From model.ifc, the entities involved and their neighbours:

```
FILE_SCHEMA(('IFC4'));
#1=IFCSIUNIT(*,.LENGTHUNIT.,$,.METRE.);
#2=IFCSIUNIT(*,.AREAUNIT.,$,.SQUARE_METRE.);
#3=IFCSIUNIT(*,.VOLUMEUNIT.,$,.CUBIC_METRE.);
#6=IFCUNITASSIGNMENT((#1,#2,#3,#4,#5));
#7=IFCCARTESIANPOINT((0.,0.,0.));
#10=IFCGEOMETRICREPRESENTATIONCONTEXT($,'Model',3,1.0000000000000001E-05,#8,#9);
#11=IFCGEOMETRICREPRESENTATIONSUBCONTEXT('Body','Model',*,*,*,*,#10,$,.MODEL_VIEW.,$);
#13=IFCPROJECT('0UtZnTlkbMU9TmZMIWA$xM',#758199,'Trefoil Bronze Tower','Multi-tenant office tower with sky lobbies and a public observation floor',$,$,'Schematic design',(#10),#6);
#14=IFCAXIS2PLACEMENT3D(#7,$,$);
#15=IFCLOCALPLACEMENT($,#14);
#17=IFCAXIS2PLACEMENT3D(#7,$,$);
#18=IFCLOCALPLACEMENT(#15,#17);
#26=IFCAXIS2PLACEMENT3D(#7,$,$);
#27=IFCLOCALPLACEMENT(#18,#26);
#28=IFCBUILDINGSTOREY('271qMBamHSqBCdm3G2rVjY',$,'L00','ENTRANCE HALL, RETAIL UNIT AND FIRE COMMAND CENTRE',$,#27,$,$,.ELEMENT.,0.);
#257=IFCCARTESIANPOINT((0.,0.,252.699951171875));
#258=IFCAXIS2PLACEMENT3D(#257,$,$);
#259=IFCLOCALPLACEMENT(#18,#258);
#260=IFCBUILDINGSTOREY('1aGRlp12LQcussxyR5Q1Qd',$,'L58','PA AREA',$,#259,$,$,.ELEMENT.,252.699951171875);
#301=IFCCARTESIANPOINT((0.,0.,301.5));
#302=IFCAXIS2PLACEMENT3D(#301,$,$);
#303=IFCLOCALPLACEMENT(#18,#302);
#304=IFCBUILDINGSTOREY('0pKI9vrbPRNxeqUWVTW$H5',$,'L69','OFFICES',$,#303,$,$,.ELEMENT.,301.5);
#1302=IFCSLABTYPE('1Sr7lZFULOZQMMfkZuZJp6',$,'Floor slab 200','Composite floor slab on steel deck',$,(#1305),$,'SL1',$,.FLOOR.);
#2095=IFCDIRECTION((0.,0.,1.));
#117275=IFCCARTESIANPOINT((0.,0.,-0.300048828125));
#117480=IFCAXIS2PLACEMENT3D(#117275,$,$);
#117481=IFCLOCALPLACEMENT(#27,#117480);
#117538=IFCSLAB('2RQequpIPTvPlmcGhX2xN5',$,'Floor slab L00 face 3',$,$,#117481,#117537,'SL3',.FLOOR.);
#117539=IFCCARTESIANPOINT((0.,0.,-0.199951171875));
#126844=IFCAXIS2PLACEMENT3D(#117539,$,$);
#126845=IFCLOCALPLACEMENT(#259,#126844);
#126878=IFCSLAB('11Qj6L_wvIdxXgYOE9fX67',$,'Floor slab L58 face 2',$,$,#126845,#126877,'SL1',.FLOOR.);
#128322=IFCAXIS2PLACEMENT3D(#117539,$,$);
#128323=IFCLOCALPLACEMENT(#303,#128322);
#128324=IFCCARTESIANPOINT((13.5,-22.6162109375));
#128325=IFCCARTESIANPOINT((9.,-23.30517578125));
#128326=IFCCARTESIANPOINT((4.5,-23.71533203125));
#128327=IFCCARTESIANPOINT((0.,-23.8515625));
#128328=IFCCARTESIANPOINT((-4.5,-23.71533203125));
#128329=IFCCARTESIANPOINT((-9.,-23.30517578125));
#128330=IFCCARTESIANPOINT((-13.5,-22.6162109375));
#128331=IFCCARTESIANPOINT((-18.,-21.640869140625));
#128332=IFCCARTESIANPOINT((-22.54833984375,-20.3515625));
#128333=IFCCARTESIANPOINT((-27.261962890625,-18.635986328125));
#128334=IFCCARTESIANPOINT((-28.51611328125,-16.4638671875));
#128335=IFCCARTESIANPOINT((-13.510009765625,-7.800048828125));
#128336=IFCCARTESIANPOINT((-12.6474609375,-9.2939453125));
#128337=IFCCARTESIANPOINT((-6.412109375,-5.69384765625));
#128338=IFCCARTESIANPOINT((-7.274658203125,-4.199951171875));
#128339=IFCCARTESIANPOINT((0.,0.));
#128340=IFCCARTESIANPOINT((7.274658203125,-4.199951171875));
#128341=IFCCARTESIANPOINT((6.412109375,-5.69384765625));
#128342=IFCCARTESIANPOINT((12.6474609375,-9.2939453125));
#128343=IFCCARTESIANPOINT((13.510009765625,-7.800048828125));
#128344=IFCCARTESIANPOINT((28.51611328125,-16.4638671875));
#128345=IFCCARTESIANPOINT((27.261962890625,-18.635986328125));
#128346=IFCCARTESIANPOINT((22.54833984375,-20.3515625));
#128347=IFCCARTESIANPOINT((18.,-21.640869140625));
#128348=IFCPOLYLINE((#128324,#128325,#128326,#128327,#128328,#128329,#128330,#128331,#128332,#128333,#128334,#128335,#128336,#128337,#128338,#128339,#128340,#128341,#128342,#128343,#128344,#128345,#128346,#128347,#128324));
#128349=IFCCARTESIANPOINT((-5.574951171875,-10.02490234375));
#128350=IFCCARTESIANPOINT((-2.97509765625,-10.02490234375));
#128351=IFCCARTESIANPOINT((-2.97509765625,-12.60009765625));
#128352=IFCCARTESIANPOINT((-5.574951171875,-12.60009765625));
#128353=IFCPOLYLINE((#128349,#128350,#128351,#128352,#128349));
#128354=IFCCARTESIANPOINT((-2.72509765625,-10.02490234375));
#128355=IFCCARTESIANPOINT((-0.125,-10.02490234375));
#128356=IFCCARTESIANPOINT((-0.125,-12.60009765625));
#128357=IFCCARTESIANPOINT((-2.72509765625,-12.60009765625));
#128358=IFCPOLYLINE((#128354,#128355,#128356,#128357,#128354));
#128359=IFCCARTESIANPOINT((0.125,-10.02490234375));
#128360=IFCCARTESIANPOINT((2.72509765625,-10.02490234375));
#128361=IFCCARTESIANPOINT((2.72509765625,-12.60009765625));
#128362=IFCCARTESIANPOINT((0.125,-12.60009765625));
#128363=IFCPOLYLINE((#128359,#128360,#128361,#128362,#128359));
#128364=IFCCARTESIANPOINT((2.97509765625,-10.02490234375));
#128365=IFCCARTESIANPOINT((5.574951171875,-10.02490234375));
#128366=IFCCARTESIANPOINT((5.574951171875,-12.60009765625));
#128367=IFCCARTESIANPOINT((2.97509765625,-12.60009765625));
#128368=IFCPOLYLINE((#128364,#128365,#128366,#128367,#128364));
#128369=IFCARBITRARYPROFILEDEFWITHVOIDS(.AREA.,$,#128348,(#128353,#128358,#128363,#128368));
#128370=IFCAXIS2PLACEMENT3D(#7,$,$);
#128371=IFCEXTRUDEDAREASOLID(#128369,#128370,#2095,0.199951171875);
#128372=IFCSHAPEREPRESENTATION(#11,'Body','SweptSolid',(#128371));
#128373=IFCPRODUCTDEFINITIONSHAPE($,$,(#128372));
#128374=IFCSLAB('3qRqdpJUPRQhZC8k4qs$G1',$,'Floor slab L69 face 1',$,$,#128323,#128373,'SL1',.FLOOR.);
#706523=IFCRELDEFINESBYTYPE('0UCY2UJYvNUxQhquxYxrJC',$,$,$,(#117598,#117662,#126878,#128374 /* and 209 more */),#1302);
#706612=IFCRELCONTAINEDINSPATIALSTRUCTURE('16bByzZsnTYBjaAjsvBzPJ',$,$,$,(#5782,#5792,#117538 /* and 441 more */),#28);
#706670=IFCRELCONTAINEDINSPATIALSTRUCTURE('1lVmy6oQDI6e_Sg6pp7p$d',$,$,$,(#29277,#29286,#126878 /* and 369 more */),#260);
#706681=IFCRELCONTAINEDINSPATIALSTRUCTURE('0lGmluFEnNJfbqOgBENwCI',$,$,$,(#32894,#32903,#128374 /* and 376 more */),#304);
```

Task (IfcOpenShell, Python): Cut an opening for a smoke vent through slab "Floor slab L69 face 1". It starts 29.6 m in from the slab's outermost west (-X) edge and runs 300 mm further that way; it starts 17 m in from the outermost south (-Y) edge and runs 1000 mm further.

```python
import numpy as np
import ifcopenshell
import ifcopenshell.api.feature
import ifcopenshell.api.geometry
import ifcopenshell.api.root
import ifcopenshell.geom
import ifcopenshell.util.placement
import ifcopenshell.util.representation
import ifcopenshell.util.shape
import ifcopenshell.util.unit

model = ifcopenshell.open("model.ifc")
unit_scale = ifcopenshell.util.unit.calculate_unit_scale(model)
settings = ifcopenshell.geom.settings()


def volume(element):
    """Net volume in cubic metres, openings subtracted."""
    shape = ifcopenshell.geom.create_shape(settings, element)
    return ifcopenshell.util.shape.get_volume(shape.geometry)


slab = model.by_id(128374)
before = volume(slab)

# Extent in the slab's own axes, in metres. The edges named are its -X and -Y sides.
slab_shape = ifcopenshell.geom.create_shape(settings, slab)
vertices = ifcopenshell.util.shape.get_vertices(slab_shape.geometry)
x_min, y_min, bottom = vertices.min(axis=0)
top = vertices[:, 2].max()

opening = ifcopenshell.api.root.create_entity(model, ifc_class="IfcOpeningElement", name="Smoke vent opening", predefined_type="OPENING")
context = ifcopenshell.util.representation.get_context(model, "Model", "Body", "MODEL_VIEW")
width, depth = 0.3, 1
outline = [(0.0, 0.0), (width, 0.0), (width, depth), (0.0, depth), (0.0, 0.0)]
# Overshoot both faces by 50 mm so the cut is clean.
shape = ifcopenshell.api.geometry.add_slab_representation(
    model, context=context, depth=top - bottom + 0.1, polyline=outline
)
ifcopenshell.api.geometry.assign_representation(model, product=opening, representation=shape)

matrix = ifcopenshell.util.placement.get_local_placement(slab.ObjectPlacement)
matrix[:, 3] = matrix @ np.append(np.array([x_min + 29.6, y_min + 17, bottom - 0.05]) / unit_scale, 1.0)
ifcopenshell.api.geometry.edit_object_placement(model, product=opening, matrix=matrix, is_si=False)
ifcopenshell.api.feature.add_feature(model, feature=opening, element=slab)

after = volume(slab)

print(f"slab volume {before:.3f} -> {after:.3f} m3")

model.write("model_edited.ifc")
```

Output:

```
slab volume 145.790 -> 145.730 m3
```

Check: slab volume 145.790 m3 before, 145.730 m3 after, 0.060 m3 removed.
